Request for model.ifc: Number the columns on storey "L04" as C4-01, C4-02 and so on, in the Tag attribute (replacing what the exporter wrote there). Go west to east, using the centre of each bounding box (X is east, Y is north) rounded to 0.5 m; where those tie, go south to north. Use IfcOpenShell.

First a look at what the model holds.

```python
import ifcopenshell
import ifcopenshell.util.element
import ifcopenshell.util.placement

model = ifcopenshell.open("model.ifc")
print(model.schema)
storey = next(s for s in model.by_type("IfcBuildingStorey") if s.Name == "L04")
columns = [e for e in ifcopenshell.util.element.get_decomposition(storey) if e.is_a("IfcColumn")]
for e in sorted(columns, key=lambda e: e.id()):
    origin = ifcopenshell.util.placement.get_local_placement(e.ObjectPlacement)[:3, 3]
    print(e.id(), e.Tag, e.Name, origin.round(2) + 0.0, sep=" | ")
```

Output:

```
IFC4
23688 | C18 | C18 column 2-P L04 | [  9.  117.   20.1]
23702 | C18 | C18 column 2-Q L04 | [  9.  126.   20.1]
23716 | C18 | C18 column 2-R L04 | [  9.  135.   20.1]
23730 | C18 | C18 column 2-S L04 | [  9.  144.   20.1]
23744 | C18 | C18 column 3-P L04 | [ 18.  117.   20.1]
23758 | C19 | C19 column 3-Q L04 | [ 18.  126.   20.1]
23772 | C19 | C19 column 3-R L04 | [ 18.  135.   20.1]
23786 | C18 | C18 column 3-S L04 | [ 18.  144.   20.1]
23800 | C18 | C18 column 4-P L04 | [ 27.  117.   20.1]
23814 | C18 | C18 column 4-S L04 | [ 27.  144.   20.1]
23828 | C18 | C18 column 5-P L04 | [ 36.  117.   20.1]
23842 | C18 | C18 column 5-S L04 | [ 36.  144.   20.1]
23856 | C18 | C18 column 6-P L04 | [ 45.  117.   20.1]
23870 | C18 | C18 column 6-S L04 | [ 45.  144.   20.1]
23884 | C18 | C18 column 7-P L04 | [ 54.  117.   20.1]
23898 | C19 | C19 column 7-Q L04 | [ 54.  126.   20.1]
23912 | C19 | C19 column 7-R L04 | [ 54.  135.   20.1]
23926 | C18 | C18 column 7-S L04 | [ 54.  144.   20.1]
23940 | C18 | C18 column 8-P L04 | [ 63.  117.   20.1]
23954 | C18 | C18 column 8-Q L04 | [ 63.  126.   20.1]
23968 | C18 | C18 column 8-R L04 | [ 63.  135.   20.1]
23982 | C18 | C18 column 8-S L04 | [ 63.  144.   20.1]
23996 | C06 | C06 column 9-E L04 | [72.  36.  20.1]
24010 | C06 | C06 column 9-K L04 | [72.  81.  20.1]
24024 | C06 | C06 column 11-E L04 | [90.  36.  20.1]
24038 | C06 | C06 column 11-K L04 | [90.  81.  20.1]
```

```python
import ifcopenshell
import ifcopenshell.geom
import ifcopenshell.util.element
import ifcopenshell.util.shape

model = ifcopenshell.open("model.ifc")
settings = ifcopenshell.geom.settings()
settings.set("use-world-coords", True)


def centre(element):
    shape = ifcopenshell.geom.create_shape(settings, element)
    return ifcopenshell.util.shape.get_bbox_centroid(shape.geometry)


storey = next(s for s in model.by_type("IfcBuildingStorey") if s.Name == "L04")
columns = [e for e in ifcopenshell.util.element.get_decomposition(storey) if e.is_a("IfcColumn")]

# Insertion points can sit at a corner or the storey origin, so sort by the geometry (in metres).
centres = {e: centre(e) for e in columns}
columns.sort(key=lambda e: (round(centres[e][0] / 0.5), centres[e][1]))

for i, e in enumerate(columns, start=1):
    number = f"C4-{i:02d}"
    e.Tag = number
    print(e.id(), number)

model.write("model_edited.ifc")
```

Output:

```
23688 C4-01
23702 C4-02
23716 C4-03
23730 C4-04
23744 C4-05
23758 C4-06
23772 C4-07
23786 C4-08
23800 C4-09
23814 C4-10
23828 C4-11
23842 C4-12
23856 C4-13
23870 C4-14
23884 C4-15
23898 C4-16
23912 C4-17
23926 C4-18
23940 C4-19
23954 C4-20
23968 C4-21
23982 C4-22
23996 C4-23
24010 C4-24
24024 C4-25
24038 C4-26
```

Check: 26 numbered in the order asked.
